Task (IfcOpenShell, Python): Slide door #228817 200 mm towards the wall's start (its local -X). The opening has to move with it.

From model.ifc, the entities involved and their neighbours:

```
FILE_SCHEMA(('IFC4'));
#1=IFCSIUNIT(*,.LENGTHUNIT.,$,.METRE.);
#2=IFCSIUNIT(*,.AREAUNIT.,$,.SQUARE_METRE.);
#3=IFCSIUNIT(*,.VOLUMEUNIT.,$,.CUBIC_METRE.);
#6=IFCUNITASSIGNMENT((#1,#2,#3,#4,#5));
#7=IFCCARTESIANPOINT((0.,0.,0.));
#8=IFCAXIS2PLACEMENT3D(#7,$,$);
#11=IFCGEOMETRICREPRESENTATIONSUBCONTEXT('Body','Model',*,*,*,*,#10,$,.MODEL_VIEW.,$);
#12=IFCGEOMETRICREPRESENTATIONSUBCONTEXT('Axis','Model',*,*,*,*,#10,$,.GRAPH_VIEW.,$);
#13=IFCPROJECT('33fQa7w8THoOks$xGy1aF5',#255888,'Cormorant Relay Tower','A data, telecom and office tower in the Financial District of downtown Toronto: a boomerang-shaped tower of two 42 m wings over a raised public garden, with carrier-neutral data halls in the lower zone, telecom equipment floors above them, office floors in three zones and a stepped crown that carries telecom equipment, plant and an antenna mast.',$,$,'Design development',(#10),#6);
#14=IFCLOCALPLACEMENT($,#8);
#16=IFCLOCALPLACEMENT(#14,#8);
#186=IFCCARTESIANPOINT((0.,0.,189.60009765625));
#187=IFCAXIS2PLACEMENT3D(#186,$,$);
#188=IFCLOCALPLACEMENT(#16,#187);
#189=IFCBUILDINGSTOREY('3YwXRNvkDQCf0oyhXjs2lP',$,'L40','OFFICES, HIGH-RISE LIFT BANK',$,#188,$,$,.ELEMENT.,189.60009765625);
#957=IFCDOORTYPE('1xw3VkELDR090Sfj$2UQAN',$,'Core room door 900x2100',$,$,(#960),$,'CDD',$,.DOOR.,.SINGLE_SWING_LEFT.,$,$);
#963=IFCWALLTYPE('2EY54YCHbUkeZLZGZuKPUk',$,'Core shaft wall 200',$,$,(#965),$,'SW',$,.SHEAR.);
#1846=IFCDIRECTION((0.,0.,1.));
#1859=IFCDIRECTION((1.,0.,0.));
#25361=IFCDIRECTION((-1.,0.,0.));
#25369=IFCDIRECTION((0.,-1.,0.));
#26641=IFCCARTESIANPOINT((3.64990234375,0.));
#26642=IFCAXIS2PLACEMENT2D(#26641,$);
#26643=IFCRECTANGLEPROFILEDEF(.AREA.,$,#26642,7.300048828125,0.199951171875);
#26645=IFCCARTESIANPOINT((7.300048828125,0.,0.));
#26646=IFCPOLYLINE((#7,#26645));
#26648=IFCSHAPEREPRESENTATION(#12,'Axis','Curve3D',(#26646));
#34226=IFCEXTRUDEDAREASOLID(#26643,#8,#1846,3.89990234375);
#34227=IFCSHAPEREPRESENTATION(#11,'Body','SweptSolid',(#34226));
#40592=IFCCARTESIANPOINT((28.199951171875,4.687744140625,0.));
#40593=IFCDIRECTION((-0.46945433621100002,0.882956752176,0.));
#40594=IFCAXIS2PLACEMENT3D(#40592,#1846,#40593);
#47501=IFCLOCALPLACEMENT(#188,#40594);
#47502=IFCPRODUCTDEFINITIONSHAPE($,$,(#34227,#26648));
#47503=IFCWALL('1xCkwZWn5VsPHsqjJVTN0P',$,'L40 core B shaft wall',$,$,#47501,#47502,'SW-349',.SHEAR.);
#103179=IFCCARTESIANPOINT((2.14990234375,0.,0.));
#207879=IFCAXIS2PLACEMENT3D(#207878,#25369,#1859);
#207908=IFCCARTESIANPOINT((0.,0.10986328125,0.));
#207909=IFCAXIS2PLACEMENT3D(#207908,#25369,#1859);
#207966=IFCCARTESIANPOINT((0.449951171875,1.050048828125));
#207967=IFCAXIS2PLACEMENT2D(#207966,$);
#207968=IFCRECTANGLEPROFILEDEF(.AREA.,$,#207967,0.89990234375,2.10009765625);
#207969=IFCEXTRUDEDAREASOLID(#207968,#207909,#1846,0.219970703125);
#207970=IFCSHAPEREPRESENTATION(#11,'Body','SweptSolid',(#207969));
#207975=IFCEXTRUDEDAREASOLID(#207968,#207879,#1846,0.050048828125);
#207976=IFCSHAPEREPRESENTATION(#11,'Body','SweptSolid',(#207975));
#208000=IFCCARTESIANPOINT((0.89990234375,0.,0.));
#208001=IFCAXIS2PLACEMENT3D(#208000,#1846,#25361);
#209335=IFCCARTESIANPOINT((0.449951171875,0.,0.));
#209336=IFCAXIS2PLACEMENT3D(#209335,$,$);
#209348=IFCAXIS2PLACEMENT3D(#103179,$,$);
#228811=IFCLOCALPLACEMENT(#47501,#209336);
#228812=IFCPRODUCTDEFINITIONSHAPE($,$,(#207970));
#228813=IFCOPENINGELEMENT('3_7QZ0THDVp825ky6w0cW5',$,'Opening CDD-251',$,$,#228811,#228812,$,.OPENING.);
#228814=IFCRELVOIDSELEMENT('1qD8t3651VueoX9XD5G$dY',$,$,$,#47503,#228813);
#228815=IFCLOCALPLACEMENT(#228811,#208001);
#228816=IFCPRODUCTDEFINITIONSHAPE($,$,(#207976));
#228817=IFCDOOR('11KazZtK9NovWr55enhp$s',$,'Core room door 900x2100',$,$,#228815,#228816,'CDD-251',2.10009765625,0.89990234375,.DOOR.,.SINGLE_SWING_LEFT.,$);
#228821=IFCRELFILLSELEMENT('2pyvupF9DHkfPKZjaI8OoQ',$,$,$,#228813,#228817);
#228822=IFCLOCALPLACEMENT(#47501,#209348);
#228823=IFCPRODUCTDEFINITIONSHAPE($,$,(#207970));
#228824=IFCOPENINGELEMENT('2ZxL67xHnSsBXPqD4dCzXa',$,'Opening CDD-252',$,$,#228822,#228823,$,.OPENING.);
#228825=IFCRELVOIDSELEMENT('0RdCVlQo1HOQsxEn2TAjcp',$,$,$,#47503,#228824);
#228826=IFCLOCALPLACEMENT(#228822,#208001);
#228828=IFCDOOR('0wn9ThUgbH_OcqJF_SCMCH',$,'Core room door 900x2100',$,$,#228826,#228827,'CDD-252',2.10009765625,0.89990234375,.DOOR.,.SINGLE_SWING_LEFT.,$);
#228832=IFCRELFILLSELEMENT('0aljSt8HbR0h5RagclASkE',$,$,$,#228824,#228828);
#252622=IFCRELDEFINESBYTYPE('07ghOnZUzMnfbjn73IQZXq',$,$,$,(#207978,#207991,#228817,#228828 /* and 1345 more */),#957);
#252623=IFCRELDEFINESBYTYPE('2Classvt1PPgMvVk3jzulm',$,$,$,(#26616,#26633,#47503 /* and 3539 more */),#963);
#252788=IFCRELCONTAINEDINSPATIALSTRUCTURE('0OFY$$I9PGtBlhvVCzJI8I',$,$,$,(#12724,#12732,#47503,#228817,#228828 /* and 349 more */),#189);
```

```python
import ifcopenshell
import ifcopenshell.api.geometry
import ifcopenshell.util.placement

model = ifcopenshell.open("model.ifc")

door = model.by_id(228817)
opening = door.FillsVoids[0].RelatingOpeningElement
wall = opening.VoidsElements[0].RelatingBuildingElement

wall_matrix = ifcopenshell.util.placement.get_local_placement(wall.ObjectPlacement)
shift = wall_matrix[:3, 0] * -0.2
before = ifcopenshell.util.placement.get_local_placement(door.ObjectPlacement)[:3, 3].copy()

# The door is placed relative to its opening, so it follows when the opening moves.
matrix = ifcopenshell.util.placement.get_local_placement(opening.ObjectPlacement)
matrix[:3, 3] += shift
ifcopenshell.api.geometry.edit_object_placement(
    model, product=opening, matrix=matrix, is_si=False, should_transform_children=True
)

after = ifcopenshell.util.placement.get_local_placement(door.ObjectPlacement)[:3, 3]
print("door moved by", (after - before).round(3) + 0.0)

model.write("model_edited.ifc")
```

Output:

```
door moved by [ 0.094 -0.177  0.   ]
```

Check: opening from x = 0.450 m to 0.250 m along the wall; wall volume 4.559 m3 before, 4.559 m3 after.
